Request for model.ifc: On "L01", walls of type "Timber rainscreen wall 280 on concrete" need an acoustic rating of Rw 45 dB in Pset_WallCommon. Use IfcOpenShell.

First a look at what the model holds.

```python
import ifcopenshell
import ifcopenshell.util.element

model = ifcopenshell.open("model.ifc")
print(model.schema)
storey = next(s for s in model.by_type("IfcBuildingStorey") if s.Name == "L01")
walls = [e for e in ifcopenshell.util.element.get_decomposition(storey) if e.is_a("IfcWall")]
seen = {}
for e in walls:
    element_type = ifcopenshell.util.element.get_type(e)
    key = (element_type.Name if element_type != e and element_type else None, ifcopenshell.util.element.get_pset(e, "Pset_WallCommon", "AcousticRating"))
    seen[key] = seen.get(key, 0) + 1
for (name, value), count in sorted(seen.items(), key=str):
    print(count, "x", name, "|", value)
```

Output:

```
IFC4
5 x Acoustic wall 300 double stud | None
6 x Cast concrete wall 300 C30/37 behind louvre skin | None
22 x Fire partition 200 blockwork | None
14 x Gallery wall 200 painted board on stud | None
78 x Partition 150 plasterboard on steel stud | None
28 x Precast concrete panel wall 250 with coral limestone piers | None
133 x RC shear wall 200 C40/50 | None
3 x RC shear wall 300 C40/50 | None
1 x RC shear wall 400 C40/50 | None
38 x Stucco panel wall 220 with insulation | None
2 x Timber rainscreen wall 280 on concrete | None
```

```python
import ifcopenshell
import ifcopenshell.api.pset
import ifcopenshell.util.element

model = ifcopenshell.open("model.ifc")

storey = next(s for s in model.by_type("IfcBuildingStorey") if s.Name == "L01")
walls = [e for e in ifcopenshell.util.element.get_decomposition(storey) if e.is_a("IfcWall")]

count = 0
for e in walls:
    element_type = ifcopenshell.util.element.get_type(e)
    if element_type in (None, e) or element_type.Name != "Timber rainscreen wall 280 on concrete":
        continue
    # add_pset returns the element's existing set when there is one.
    pset = ifcopenshell.api.pset.add_pset(model, product=e, name="Pset_WallCommon")
    ifcopenshell.api.pset.edit_pset(model, pset=pset, properties={"AcousticRating": "Rw 45 dB"})
    count += 1

print(count, "walls updated")

model.write("model_updated.ifc")
```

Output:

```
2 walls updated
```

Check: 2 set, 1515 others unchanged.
